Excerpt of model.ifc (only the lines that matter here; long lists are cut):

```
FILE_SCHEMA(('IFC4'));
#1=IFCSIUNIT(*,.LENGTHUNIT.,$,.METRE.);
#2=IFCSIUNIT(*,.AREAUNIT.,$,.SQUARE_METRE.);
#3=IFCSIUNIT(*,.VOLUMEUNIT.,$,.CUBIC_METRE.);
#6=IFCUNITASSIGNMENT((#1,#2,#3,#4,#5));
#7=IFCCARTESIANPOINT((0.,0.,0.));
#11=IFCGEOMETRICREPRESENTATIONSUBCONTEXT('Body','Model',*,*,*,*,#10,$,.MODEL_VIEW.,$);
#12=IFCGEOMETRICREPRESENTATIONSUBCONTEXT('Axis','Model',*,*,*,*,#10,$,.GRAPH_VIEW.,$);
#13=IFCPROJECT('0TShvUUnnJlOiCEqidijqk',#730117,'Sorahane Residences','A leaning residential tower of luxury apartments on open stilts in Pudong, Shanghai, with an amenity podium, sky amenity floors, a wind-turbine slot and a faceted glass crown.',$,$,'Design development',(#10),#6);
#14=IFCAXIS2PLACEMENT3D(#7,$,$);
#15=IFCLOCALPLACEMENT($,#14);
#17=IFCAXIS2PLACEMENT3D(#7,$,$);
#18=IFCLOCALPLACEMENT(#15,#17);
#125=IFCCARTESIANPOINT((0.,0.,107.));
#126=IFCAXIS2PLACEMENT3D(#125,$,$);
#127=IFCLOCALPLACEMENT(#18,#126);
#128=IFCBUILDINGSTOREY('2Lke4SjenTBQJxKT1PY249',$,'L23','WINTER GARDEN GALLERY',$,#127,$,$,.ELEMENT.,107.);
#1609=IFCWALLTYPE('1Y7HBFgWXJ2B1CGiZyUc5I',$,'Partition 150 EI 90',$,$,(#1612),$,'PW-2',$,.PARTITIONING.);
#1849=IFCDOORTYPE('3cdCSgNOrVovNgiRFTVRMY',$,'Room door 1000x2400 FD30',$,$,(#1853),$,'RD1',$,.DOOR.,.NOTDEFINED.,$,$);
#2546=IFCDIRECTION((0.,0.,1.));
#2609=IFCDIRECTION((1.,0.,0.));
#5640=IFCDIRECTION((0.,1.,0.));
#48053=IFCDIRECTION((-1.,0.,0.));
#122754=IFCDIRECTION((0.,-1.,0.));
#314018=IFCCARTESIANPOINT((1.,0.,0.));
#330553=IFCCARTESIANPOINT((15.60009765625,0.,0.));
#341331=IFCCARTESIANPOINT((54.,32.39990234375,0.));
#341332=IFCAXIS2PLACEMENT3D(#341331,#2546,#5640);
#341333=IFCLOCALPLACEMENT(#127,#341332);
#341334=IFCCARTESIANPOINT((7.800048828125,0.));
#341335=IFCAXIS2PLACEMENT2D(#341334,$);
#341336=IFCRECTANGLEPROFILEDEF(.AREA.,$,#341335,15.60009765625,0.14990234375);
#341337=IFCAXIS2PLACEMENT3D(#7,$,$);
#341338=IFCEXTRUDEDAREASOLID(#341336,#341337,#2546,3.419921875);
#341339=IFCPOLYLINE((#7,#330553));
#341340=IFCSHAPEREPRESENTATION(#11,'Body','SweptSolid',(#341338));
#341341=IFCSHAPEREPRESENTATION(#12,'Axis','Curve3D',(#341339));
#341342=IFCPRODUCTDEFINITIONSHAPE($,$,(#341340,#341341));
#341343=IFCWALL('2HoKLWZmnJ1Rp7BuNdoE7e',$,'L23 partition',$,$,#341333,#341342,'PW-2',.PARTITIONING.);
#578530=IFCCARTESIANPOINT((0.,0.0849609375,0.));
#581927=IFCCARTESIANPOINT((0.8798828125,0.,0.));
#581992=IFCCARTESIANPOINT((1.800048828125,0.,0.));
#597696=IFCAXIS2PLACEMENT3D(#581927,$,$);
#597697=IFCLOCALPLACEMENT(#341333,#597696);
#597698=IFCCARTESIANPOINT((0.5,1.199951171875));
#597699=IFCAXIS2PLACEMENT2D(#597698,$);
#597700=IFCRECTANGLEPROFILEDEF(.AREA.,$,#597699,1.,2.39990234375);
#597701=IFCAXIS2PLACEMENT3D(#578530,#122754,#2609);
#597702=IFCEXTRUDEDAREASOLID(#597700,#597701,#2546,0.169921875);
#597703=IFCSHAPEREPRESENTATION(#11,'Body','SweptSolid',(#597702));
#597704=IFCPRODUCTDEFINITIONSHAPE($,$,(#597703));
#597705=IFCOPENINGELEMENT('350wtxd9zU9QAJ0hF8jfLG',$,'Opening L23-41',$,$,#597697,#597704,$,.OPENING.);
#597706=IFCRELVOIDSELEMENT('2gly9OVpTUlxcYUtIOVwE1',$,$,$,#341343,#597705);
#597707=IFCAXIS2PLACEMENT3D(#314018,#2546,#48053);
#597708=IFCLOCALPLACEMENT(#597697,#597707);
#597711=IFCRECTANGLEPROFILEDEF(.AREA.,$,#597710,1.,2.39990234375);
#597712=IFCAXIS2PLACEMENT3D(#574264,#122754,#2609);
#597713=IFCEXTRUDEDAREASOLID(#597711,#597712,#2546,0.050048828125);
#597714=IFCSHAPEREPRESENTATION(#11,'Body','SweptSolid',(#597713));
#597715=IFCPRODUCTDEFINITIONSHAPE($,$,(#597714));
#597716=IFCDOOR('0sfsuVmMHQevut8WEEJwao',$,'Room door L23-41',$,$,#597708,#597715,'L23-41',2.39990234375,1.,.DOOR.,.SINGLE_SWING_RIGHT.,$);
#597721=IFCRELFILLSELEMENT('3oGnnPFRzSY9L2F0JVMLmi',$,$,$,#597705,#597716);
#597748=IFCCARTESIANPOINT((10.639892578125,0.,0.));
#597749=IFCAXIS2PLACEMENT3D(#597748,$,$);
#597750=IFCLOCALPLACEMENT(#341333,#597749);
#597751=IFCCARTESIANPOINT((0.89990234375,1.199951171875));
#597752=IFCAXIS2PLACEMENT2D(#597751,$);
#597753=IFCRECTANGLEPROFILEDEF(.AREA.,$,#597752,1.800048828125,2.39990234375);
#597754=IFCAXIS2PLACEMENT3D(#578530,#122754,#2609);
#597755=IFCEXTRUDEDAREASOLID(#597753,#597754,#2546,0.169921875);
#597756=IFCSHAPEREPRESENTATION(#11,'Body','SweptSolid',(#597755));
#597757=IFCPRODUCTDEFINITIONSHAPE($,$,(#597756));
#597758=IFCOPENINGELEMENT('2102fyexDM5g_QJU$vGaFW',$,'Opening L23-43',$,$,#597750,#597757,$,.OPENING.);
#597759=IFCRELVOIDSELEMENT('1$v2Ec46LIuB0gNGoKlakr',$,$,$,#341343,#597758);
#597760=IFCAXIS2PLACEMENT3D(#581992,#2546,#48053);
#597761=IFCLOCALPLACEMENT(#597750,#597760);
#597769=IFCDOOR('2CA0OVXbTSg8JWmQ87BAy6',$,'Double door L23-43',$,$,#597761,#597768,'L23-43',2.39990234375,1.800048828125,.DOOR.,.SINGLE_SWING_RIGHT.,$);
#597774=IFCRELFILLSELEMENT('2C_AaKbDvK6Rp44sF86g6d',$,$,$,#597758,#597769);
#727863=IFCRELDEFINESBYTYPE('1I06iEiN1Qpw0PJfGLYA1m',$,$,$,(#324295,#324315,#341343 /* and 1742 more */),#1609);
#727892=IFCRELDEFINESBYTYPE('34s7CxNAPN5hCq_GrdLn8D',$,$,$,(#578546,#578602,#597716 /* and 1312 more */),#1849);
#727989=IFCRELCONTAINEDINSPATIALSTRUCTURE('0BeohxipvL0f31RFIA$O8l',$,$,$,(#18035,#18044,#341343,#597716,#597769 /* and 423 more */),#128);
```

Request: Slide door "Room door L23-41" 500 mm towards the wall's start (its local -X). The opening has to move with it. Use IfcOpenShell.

```python
import ifcopenshell
import ifcopenshell.api.geometry
import ifcopenshell.util.placement
import ifcopenshell.util.unit

model = ifcopenshell.open("model.ifc")
unit_scale = ifcopenshell.util.unit.calculate_unit_scale(model)

door = model.by_id(597716)
opening = door.FillsVoids[0].RelatingOpeningElement
wall = opening.VoidsElements[0].RelatingBuildingElement

wall_matrix = ifcopenshell.util.placement.get_local_placement(wall.ObjectPlacement)
shift = wall_matrix[:3, 0] * -0.5 / unit_scale
before = ifcopenshell.util.placement.get_local_placement(door.ObjectPlacement)[:3, 3].copy()

# The door is placed relative to its opening, so it follows when the opening moves.
matrix = ifcopenshell.util.placement.get_local_placement(opening.ObjectPlacement)
matrix[:3, 3] += shift
ifcopenshell.api.geometry.edit_object_placement(
    model, product=opening, matrix=matrix, is_si=False, should_transform_children=True
)

after = ifcopenshell.util.placement.get_local_placement(door.ObjectPlacement)[:3, 3]
print("door moved by", (after - before).round(3) + 0.0)

model.write("model_rev.ifc")
```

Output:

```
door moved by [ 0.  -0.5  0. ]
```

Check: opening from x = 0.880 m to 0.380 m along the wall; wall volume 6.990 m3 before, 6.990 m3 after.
